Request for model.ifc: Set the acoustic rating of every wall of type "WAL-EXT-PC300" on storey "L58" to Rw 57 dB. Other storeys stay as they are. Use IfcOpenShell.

First a look at what the model holds.

```python
import ifcopenshell
import ifcopenshell.util.element

model = ifcopenshell.open("model.ifc")
print(model.schema)
storey = next(s for s in model.by_type("IfcBuildingStorey") if s.Name == "L58")
walls = [e for e in ifcopenshell.util.element.get_decomposition(storey) if e.is_a("IfcWall")]
seen = {}
for e in walls:
    element_type = ifcopenshell.util.element.get_type(e)
    key = (element_type.Name if element_type != e and element_type else None, ifcopenshell.util.element.get_pset(e, "Pset_WallCommon", "AcousticRating"))
    seen[key] = seen.get(key, 0) + 1
for (name, value), count in sorted(seen.items(), key=str):
    print(count, "x", name, "|", value)
```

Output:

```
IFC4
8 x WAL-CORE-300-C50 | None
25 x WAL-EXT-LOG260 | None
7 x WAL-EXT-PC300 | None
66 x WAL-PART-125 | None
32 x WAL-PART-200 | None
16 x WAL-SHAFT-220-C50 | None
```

```python
import ifcopenshell
import ifcopenshell.api.pset
import ifcopenshell.util.element

model = ifcopenshell.open("model.ifc")

storey = next(s for s in model.by_type("IfcBuildingStorey") if s.Name == "L58")
walls = [e for e in ifcopenshell.util.element.get_decomposition(storey) if e.is_a("IfcWall")]

count = 0
for e in walls:
    element_type = ifcopenshell.util.element.get_type(e)
    if element_type in (None, e) or element_type.Name != "WAL-EXT-PC300":
        continue
    found = ifcopenshell.util.element.get_pset(e, "Pset_WallCommon", should_inherit=False)
    if found:
        pset = model.by_id(found["id"])
        if len(ifcopenshell.util.element.get_elements_by_pset(pset)) > 1:
            pset = ifcopenshell.api.pset.unshare_pset(model, products=[e], pset=pset)[0]
    else:
        pset = ifcopenshell.api.pset.add_pset(model, product=e, name="Pset_WallCommon")
    ifcopenshell.api.pset.edit_pset(model, pset=pset, properties={"AcousticRating": "Rw 57 dB"})
    count += 1

print(count, "walls updated")

model.write("model_updated.ifc")
```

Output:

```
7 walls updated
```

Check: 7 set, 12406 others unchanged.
